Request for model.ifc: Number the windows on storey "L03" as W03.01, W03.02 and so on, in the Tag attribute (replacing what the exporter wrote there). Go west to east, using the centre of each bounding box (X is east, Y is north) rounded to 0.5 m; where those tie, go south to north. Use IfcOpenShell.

First a look at what the model holds.

```python
import ifcopenshell
import ifcopenshell.util.element
import ifcopenshell.util.placement

model = ifcopenshell.open("model.ifc")
print(model.schema)
storey = next(s for s in model.by_type("IfcBuildingStorey") if s.Name == "L03")
windows = [e for e in ifcopenshell.util.element.get_decomposition(storey) if e.is_a("IfcWindow")]
for e in sorted(windows, key=lambda e: e.id()):
    origin = ifcopenshell.util.placement.get_local_placement(e.ObjectPlacement)[:3, 3]
    print(e.id(), e.Tag, e.Name, origin.round(2) + 0.0, sep=" | ")
```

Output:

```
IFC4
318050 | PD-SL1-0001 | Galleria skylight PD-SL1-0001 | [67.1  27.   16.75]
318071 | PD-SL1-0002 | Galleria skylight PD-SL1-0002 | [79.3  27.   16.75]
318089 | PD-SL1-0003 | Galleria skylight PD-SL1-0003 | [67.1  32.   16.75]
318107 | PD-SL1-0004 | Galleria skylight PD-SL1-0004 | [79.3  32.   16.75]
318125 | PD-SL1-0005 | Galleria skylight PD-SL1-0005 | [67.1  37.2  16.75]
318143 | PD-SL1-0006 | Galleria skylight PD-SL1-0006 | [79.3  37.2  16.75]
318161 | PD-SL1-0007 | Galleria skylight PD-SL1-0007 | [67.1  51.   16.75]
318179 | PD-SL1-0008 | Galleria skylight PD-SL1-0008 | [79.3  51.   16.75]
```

```python
import ifcopenshell
import ifcopenshell.geom
import ifcopenshell.util.element
import ifcopenshell.util.shape

model = ifcopenshell.open("model.ifc")
settings = ifcopenshell.geom.settings()
settings.set("use-world-coords", True)


def centre(element):
    shape = ifcopenshell.geom.create_shape(settings, element)
    return ifcopenshell.util.shape.get_bbox_centroid(shape.geometry)


storey = next(s for s in model.by_type("IfcBuildingStorey") if s.Name == "L03")
windows = [e for e in ifcopenshell.util.element.get_decomposition(storey) if e.is_a("IfcWindow")]

# Insertion points can sit at a corner or the storey origin, so sort by the geometry (in metres).
centres = {e: centre(e) for e in windows}
windows.sort(key=lambda e: (round(centres[e][0] / 0.5), centres[e][1]))

for i, e in enumerate(windows, start=1):
    number = f"W03.{i:02d}"
    e.Tag = number
    print(e.id(), number)

model.write("model_edited.ifc")
```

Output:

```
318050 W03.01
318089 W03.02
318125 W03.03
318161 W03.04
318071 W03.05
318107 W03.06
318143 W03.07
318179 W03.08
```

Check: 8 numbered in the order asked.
